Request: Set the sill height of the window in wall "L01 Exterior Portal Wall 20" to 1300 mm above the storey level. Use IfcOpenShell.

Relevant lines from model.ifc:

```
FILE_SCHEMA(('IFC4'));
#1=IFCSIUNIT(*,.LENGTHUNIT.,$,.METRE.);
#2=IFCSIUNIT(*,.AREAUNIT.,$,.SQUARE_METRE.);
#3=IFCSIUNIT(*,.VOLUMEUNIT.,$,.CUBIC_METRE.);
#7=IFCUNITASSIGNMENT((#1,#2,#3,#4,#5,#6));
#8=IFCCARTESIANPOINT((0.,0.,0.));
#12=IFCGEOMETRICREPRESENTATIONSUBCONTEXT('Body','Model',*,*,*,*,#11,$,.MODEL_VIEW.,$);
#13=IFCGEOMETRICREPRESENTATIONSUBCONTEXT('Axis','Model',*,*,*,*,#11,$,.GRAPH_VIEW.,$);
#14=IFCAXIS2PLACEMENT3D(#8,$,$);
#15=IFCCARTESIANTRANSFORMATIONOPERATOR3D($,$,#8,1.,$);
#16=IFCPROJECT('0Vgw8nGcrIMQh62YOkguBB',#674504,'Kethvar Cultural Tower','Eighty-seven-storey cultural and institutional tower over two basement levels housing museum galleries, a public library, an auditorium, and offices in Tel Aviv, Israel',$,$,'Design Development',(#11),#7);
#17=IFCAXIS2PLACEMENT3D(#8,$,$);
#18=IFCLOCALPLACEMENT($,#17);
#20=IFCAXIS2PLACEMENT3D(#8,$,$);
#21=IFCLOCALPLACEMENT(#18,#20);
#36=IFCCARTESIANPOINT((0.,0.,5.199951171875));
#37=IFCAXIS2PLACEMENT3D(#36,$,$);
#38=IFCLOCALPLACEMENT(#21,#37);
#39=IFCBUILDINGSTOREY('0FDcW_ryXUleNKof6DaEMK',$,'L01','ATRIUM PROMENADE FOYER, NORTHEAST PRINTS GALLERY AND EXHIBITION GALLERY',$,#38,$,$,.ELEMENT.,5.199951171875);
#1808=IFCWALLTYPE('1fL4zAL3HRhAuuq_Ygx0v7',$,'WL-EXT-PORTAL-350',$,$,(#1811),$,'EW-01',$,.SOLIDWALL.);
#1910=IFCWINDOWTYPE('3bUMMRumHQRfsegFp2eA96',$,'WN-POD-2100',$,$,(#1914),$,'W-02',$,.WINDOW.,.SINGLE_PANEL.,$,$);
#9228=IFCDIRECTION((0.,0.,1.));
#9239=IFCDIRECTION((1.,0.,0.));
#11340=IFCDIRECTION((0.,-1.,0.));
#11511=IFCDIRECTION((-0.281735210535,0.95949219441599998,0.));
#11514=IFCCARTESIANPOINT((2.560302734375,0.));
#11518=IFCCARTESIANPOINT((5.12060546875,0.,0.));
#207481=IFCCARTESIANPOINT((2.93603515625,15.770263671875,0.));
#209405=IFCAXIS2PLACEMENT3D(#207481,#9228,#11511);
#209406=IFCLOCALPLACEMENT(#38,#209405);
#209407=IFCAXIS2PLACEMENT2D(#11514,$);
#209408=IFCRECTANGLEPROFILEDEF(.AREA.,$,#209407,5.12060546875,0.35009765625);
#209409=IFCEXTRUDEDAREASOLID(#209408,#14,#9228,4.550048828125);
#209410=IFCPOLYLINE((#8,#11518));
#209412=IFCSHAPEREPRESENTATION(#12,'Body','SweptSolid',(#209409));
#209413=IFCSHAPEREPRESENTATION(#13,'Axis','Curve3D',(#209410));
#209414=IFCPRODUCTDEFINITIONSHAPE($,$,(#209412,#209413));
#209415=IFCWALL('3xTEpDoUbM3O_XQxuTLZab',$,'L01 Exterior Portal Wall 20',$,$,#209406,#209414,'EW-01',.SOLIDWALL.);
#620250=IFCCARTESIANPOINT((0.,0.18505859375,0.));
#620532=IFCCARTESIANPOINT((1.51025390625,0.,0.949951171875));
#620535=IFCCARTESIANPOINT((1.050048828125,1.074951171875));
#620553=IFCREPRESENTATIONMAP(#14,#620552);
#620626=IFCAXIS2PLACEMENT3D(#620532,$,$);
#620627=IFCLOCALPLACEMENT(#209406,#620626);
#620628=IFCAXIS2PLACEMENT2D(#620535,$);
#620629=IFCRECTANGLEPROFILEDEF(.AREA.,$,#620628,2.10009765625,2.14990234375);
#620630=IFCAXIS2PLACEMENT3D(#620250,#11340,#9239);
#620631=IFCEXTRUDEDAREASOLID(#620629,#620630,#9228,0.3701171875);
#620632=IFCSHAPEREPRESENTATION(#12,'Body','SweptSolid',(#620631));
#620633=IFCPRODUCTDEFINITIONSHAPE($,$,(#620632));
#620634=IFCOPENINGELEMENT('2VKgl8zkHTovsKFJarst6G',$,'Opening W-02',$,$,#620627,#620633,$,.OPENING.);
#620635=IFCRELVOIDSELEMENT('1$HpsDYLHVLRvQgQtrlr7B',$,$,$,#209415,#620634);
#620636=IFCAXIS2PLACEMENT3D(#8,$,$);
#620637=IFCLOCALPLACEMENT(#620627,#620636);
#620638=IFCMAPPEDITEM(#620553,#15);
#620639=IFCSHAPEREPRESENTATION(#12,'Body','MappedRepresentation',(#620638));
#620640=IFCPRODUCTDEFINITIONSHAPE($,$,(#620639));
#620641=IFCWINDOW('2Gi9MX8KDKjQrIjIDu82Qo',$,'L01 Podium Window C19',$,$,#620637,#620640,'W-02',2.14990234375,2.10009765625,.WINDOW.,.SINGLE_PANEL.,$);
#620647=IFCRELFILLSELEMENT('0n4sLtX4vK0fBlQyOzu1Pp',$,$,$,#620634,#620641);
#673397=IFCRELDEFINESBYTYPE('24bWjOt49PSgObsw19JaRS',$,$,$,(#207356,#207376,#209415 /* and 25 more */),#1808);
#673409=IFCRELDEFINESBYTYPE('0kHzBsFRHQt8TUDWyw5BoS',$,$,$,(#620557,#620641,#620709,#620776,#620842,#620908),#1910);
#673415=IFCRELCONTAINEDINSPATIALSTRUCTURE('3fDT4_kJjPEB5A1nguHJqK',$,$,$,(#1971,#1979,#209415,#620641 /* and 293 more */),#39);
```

```python
import numpy as np
import ifcopenshell
import ifcopenshell.api.geometry
import ifcopenshell.geom
import ifcopenshell.util.element
import ifcopenshell.util.placement
import ifcopenshell.util.shape
import ifcopenshell.util.unit

model = ifcopenshell.open("model.ifc")
unit_scale = ifcopenshell.util.unit.calculate_unit_scale(model)

window = model.by_id(620641)
opening = window.FillsVoids[0].RelatingOpeningElement
storey = ifcopenshell.util.element.get_container(window, ifc_class="IfcBuildingStorey")
level = ifcopenshell.util.placement.get_local_placement(storey.ObjectPlacement)[2, 3]

# The opening's origin need not be at the sill, so measure its lowest point.
shape = ifcopenshell.geom.create_shape(ifcopenshell.geom.settings(), opening)
bottom = ifcopenshell.util.shape.get_shape_bottom_elevation(shape, shape.geometry) / unit_scale
dz = level + 1.3 / unit_scale - bottom

shift = np.array([0.0, 0.0, dz])
# The window is placed relative to its opening, so it follows when the opening moves.
matrix = ifcopenshell.util.placement.get_local_placement(opening.ObjectPlacement)
matrix[:3, 3] += shift
ifcopenshell.api.geometry.edit_object_placement(
    model, product=opening, matrix=matrix, is_si=False, should_transform_children=True
)

print(f"moved by {dz * unit_scale:+.3f} m")

model.write("model-out.ifc")
```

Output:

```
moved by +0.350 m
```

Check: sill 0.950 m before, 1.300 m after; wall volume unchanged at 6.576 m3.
